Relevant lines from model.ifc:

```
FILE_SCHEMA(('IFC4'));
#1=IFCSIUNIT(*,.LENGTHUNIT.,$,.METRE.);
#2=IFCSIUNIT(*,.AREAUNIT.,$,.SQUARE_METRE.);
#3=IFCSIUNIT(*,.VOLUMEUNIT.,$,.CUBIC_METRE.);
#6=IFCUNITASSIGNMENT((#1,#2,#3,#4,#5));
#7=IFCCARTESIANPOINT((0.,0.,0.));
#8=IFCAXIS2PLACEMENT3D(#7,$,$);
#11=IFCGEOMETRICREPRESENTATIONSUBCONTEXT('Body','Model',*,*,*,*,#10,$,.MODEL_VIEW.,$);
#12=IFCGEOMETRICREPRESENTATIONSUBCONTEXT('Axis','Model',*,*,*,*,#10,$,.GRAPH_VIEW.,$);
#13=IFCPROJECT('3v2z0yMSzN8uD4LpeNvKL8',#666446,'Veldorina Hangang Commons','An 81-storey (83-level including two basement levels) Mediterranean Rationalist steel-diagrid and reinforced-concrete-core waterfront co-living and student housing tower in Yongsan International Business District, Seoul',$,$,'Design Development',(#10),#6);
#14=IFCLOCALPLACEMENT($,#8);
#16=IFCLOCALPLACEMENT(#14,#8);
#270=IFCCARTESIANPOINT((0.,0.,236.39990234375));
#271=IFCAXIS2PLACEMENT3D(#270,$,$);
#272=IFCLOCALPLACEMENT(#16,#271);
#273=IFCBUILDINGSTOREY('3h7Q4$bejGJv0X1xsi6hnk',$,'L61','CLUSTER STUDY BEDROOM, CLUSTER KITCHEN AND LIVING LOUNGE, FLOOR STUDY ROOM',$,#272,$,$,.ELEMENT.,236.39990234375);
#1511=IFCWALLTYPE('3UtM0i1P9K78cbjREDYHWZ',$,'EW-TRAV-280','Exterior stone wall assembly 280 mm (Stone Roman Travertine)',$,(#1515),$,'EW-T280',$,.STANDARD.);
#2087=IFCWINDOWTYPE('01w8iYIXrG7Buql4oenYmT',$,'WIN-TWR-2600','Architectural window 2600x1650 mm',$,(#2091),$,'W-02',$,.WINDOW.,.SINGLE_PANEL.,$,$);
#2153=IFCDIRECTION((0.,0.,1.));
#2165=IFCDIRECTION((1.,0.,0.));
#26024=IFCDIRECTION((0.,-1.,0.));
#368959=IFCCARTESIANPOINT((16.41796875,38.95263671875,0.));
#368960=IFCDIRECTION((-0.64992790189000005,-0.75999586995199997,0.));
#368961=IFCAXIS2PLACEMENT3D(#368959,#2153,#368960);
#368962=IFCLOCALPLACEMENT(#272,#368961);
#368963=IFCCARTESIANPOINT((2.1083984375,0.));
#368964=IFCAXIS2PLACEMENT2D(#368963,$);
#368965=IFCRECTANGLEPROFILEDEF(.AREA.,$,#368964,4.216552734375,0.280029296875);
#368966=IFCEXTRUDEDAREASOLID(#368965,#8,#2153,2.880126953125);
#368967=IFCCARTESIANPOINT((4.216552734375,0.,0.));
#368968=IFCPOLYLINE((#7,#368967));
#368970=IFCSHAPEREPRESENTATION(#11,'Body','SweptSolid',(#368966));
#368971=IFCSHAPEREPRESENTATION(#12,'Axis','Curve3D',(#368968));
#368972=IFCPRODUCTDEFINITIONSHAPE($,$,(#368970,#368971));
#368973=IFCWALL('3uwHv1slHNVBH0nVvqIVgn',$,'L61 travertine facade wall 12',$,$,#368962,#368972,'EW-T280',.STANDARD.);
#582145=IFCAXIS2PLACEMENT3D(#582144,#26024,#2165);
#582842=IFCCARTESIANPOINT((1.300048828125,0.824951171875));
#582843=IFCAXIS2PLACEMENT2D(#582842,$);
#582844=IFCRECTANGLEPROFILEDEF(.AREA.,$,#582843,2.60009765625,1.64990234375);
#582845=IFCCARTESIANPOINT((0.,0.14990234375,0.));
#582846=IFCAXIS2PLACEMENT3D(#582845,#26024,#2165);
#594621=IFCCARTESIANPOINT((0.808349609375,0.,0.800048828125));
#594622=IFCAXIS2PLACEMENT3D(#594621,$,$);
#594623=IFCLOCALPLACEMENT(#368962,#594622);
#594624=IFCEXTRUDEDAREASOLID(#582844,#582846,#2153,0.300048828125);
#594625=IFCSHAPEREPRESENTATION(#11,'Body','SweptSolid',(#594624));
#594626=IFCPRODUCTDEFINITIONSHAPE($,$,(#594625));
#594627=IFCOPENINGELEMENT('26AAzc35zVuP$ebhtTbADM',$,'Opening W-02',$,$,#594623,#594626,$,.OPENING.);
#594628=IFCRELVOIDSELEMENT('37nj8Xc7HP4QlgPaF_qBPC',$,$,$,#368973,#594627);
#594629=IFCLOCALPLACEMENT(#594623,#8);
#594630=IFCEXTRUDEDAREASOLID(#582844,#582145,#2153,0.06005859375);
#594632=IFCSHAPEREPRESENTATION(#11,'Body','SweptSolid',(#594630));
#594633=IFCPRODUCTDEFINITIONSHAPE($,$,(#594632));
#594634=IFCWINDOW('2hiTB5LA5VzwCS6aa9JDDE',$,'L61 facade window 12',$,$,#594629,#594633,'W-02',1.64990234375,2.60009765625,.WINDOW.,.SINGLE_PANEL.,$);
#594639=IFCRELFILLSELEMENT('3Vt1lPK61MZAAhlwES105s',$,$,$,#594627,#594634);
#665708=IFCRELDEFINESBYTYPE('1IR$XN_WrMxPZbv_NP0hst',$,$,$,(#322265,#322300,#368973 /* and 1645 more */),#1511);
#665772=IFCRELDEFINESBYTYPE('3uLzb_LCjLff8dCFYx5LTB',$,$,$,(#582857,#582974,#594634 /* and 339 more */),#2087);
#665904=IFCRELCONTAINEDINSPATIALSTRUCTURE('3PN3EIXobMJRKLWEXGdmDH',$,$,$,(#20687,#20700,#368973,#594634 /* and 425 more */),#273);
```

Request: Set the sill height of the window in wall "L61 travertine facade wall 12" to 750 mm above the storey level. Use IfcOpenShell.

```python
import numpy as np
import ifcopenshell
import ifcopenshell.api.geometry
import ifcopenshell.geom
import ifcopenshell.util.element
import ifcopenshell.util.placement
import ifcopenshell.util.shape
import ifcopenshell.util.unit

model = ifcopenshell.open("model.ifc")
unit_scale = ifcopenshell.util.unit.calculate_unit_scale(model)

window = model.by_guid("2hiTB5LA5VzwCS6aa9JDDE")
opening = window.FillsVoids[0].RelatingOpeningElement
storey = ifcopenshell.util.element.get_container(window, ifc_class="IfcBuildingStorey")
level = ifcopenshell.util.placement.get_local_placement(storey.ObjectPlacement)[2, 3]

# The opening's origin need not be at the sill, so measure its lowest point.
shape = ifcopenshell.geom.create_shape(ifcopenshell.geom.settings(), opening)
bottom = ifcopenshell.util.shape.get_shape_bottom_elevation(shape, shape.geometry) / unit_scale
dz = level + 0.75 - bottom

shift = np.array([0.0, 0.0, dz])
# The window is placed relative to its opening, so it follows when the opening moves.
matrix = ifcopenshell.util.placement.get_local_placement(opening.ObjectPlacement)
matrix[:3, 3] += shift
ifcopenshell.api.geometry.edit_object_placement(
    model, product=opening, matrix=matrix, is_si=False, should_transform_children=True
)

print(f"moved by {dz * unit_scale:+.3f} m")

model.write("model_v2.ifc")
```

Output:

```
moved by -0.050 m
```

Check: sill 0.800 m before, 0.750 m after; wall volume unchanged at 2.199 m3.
